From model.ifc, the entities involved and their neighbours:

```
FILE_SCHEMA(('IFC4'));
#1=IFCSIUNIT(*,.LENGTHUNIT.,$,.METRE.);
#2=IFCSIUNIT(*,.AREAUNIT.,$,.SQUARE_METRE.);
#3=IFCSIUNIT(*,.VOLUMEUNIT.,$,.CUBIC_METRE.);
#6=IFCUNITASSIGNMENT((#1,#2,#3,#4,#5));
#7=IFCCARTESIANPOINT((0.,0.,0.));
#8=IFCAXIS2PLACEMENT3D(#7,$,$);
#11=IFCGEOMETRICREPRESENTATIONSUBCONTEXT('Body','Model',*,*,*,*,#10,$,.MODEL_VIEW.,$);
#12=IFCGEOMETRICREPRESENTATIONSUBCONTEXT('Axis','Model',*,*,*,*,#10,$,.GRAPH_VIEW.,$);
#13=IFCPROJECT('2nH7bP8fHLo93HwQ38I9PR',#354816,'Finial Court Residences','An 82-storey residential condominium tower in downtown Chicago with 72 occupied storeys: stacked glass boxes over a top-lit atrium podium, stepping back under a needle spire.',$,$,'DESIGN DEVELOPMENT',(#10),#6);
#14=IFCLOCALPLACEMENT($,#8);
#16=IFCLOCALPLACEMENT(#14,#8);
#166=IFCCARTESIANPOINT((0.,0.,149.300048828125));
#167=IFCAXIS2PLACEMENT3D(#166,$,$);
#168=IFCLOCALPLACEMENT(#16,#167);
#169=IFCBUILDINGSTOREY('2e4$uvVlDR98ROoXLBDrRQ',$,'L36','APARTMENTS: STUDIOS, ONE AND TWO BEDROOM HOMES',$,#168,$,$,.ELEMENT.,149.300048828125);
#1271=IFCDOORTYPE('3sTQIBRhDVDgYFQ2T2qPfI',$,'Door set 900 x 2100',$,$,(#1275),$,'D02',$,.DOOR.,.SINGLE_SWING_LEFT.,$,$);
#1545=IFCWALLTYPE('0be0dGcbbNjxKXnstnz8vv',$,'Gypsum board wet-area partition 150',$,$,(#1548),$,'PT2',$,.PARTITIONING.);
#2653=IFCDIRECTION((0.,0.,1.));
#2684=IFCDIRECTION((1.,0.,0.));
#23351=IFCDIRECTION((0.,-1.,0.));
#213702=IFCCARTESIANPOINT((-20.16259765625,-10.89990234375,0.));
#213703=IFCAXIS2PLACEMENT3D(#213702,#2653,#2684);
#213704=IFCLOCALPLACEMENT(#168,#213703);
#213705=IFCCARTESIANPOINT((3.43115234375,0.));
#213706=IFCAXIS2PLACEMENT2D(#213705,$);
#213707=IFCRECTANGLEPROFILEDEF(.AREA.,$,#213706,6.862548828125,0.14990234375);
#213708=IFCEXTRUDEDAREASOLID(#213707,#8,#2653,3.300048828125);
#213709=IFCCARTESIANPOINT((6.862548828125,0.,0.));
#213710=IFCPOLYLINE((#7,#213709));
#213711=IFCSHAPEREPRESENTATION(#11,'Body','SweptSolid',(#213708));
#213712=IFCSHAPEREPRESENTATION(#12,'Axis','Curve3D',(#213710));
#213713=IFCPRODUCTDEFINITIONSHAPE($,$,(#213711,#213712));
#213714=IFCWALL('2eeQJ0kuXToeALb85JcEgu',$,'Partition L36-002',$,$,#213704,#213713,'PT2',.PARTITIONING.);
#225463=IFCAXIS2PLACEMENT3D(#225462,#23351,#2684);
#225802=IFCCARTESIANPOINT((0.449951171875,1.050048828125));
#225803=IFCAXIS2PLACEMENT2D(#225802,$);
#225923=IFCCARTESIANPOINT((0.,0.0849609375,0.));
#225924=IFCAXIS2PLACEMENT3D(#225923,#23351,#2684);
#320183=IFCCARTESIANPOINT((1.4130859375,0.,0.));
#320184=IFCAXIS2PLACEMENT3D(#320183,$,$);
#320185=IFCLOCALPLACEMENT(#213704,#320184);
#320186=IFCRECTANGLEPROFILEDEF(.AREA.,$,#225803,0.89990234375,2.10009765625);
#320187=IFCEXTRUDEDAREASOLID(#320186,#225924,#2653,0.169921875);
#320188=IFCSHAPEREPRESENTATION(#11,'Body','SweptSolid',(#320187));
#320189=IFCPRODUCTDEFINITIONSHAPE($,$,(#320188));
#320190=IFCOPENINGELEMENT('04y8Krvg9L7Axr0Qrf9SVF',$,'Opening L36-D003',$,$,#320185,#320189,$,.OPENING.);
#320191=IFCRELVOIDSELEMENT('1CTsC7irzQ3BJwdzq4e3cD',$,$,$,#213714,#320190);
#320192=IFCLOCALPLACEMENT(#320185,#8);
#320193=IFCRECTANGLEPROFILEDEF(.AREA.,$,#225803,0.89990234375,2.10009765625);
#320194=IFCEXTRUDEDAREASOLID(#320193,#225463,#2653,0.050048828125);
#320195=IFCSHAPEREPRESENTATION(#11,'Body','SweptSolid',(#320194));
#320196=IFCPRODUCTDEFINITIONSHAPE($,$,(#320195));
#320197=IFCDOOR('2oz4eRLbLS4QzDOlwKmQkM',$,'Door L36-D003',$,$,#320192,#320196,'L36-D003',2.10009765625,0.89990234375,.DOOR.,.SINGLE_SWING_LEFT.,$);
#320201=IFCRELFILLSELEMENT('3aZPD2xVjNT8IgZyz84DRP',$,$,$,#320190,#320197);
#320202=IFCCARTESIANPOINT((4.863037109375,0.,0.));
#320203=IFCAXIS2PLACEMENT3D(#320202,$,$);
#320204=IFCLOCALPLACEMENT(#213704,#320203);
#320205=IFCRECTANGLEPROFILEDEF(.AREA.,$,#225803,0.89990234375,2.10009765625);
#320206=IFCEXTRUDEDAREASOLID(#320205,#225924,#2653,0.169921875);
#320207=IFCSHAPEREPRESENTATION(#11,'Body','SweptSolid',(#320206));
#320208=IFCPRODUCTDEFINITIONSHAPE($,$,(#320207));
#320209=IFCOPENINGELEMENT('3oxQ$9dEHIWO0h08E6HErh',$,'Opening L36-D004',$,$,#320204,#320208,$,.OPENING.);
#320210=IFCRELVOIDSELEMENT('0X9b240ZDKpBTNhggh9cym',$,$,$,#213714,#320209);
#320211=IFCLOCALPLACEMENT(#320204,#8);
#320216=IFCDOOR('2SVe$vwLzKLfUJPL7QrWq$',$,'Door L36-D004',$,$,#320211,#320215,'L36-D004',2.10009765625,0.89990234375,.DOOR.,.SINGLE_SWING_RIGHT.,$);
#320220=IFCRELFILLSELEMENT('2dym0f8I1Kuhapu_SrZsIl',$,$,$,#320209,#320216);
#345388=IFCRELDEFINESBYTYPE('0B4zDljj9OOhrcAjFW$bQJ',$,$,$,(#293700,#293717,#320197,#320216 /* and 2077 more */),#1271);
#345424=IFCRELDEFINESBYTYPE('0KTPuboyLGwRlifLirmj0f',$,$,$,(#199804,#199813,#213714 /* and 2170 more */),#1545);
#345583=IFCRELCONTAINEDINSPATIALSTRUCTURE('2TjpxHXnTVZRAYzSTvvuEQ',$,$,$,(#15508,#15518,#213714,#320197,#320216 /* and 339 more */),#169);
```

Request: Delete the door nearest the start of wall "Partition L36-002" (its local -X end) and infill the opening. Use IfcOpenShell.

```python
import ifcopenshell
import ifcopenshell.api.feature
import ifcopenshell.api.root
import ifcopenshell.geom
import ifcopenshell.util.shape

model = ifcopenshell.open("model.ifc")
settings = ifcopenshell.geom.settings()


def volume(element):
    """Net volume in cubic metres, openings subtracted."""
    shape = ifcopenshell.geom.create_shape(settings, element)
    return ifcopenshell.util.shape.get_volume(shape.geometry)


door = model.by_id(320197)
opening = door.FillsVoids[0].RelatingOpeningElement
wall = opening.VoidsElements[0].RelatingBuildingElement
before = volume(wall)

ifcopenshell.api.root.remove_product(model, product=door)
ifcopenshell.api.feature.remove_feature(model, feature=opening)

after = volume(wall)

print(f"wall volume {before:.3f} -> {after:.3f} m3")

model.write("model_v2.ifc")
```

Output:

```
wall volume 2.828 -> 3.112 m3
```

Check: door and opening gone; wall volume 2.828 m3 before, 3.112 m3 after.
